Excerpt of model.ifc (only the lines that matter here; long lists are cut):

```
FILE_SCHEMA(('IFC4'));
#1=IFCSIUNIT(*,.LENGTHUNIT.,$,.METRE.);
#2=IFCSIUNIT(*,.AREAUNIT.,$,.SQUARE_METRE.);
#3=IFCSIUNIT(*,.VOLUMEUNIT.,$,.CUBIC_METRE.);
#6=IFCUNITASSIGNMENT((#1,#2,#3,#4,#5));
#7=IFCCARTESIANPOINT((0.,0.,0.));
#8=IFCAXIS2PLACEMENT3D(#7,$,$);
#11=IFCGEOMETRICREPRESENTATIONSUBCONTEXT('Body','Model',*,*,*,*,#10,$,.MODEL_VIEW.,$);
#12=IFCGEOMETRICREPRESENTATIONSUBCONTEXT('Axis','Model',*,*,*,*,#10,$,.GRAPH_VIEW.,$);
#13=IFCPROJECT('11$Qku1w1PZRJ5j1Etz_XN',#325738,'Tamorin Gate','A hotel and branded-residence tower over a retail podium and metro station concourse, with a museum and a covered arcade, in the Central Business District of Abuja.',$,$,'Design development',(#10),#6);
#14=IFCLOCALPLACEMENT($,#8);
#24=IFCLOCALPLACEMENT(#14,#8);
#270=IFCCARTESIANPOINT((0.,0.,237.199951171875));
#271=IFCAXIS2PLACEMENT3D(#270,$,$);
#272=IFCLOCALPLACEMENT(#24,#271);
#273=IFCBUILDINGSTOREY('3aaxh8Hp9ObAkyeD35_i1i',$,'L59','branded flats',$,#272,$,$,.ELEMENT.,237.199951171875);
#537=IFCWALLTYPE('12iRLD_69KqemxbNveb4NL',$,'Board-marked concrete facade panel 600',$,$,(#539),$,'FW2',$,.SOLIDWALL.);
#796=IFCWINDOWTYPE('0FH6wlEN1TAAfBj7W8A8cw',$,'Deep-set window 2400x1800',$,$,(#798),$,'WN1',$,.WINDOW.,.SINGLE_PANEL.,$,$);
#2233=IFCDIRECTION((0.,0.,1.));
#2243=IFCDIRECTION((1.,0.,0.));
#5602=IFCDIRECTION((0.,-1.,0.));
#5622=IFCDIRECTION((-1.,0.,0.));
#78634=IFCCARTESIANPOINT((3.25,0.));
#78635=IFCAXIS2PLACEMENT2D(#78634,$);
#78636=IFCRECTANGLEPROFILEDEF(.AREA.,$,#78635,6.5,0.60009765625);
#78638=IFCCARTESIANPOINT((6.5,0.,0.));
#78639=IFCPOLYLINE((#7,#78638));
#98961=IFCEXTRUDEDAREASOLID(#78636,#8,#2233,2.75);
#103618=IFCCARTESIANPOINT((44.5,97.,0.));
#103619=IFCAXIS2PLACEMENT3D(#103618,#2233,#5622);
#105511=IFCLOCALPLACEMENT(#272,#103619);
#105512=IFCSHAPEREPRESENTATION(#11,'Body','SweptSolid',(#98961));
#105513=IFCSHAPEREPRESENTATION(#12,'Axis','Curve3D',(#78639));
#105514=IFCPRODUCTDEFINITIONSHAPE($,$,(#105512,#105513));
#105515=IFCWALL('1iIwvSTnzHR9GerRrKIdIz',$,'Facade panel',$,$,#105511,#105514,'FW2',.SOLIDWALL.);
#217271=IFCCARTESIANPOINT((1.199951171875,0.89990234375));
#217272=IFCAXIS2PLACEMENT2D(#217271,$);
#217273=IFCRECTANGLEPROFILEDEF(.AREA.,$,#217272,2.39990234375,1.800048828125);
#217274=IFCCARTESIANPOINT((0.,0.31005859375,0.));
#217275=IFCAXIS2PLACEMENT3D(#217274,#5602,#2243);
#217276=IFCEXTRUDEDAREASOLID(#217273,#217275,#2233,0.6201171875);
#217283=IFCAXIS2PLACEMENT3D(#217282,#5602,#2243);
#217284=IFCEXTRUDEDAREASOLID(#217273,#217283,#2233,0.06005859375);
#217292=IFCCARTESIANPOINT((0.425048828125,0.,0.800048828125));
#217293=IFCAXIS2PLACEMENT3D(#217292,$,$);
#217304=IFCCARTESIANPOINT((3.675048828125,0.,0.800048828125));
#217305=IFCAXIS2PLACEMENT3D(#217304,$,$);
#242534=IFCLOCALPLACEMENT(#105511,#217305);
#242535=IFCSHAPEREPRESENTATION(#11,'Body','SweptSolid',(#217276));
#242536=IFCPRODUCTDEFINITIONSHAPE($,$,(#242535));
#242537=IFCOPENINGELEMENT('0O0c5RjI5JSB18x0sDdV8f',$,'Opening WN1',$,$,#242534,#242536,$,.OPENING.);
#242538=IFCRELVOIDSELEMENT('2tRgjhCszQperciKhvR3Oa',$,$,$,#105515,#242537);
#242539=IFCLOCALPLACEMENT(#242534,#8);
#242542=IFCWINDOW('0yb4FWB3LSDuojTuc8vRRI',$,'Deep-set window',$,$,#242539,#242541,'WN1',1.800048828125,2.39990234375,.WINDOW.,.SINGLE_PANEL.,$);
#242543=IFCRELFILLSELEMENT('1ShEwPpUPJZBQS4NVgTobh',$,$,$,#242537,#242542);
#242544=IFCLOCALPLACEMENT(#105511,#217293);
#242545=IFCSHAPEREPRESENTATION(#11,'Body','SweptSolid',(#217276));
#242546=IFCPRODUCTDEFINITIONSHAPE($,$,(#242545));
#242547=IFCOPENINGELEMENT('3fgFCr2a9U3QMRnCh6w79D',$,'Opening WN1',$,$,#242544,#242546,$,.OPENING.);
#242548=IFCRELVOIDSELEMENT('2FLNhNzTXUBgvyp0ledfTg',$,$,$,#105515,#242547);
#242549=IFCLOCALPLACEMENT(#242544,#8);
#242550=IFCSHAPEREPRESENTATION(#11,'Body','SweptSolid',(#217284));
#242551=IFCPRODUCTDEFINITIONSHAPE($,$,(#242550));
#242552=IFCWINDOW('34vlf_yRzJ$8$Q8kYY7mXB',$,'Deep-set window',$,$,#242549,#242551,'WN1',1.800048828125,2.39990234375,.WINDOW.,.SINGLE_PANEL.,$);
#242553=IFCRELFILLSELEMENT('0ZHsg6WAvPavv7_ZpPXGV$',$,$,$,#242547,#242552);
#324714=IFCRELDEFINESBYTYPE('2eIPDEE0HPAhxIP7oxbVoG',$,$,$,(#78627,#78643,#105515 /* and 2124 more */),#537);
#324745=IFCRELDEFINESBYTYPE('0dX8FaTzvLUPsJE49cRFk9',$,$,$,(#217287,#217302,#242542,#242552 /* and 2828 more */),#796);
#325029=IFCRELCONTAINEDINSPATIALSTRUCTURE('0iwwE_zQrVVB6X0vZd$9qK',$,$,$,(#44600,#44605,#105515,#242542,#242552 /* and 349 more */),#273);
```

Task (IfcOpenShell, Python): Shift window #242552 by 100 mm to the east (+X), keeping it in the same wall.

```python
import ifcopenshell
import ifcopenshell.api.geometry
import ifcopenshell.util.placement

model = ifcopenshell.open("model.ifc")

window = model.by_guid("34vlf_yRzJ$8$Q8kYY7mXB")
opening = window.FillsVoids[0].RelatingOpeningElement
wall = opening.VoidsElements[0].RelatingBuildingElement

wall_matrix = ifcopenshell.util.placement.get_local_placement(wall.ObjectPlacement)
shift = wall_matrix[:3, 0] * -0.1
before = ifcopenshell.util.placement.get_local_placement(window.ObjectPlacement)[:3, 3].copy()

# The window is placed relative to its opening, so it follows when the opening moves.
matrix = ifcopenshell.util.placement.get_local_placement(opening.ObjectPlacement)
matrix[:3, 3] += shift
ifcopenshell.api.geometry.edit_object_placement(
    model, product=opening, matrix=matrix, is_si=False, should_transform_children=True
)

after = ifcopenshell.util.placement.get_local_placement(window.ObjectPlacement)[:3, 3]
print("window moved by", (after - before).round(3) + 0.0)

model.write("model_v2.ifc")
```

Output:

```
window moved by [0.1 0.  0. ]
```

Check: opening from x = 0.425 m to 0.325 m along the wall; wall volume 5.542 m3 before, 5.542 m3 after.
